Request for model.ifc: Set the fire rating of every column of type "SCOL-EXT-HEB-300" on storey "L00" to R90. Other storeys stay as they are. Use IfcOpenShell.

First a look at what the model holds.

```python
import ifcopenshell
import ifcopenshell.util.element

model = ifcopenshell.open("model.ifc")
print(model.schema)
storey = next(s for s in model.by_type("IfcBuildingStorey") if s.Name == "L00")
columns = [e for e in ifcopenshell.util.element.get_decomposition(storey) if e.is_a("IfcColumn")]
seen = {}
for e in columns:
    element_type = ifcopenshell.util.element.get_type(e)
    key = (element_type.Name if element_type != e and element_type else None, ifcopenshell.util.element.get_pset(e, "Pset_ColumnCommon", "FireRating"))
    seen[key] = seen.get(key, 0) + 1
for (name, value), count in sorted(seen.items(), key=str):
    print(count, "x", name, "|", value)
```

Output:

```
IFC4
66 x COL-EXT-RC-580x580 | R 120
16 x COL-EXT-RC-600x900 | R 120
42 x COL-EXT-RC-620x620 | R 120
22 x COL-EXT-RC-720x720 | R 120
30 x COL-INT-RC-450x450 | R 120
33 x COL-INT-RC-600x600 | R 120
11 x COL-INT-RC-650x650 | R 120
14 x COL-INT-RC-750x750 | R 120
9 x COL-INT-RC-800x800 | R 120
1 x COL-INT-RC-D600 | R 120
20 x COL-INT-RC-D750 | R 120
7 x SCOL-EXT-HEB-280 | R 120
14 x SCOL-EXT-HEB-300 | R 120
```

```python
import ifcopenshell
import ifcopenshell.api.pset
import ifcopenshell.util.element

model = ifcopenshell.open("model.ifc")

storey = next(s for s in model.by_type("IfcBuildingStorey") if s.Name == "L00")
columns = [e for e in ifcopenshell.util.element.get_decomposition(storey) if e.is_a("IfcColumn")]

count = 0
for e in columns:
    element_type = ifcopenshell.util.element.get_type(e)
    if element_type in (None, e) or element_type.Name != "SCOL-EXT-HEB-300":
        continue
    # add_pset returns the element's existing set when there is one.
    pset = ifcopenshell.api.pset.add_pset(model, product=e, name="Pset_ColumnCommon")
    ifcopenshell.api.pset.edit_pset(model, pset=pset, properties={"FireRating": "R90"})
    count += 1

print(count, "columns updated")

model.write("model-out.ifc")
```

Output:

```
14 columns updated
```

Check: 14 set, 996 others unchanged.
